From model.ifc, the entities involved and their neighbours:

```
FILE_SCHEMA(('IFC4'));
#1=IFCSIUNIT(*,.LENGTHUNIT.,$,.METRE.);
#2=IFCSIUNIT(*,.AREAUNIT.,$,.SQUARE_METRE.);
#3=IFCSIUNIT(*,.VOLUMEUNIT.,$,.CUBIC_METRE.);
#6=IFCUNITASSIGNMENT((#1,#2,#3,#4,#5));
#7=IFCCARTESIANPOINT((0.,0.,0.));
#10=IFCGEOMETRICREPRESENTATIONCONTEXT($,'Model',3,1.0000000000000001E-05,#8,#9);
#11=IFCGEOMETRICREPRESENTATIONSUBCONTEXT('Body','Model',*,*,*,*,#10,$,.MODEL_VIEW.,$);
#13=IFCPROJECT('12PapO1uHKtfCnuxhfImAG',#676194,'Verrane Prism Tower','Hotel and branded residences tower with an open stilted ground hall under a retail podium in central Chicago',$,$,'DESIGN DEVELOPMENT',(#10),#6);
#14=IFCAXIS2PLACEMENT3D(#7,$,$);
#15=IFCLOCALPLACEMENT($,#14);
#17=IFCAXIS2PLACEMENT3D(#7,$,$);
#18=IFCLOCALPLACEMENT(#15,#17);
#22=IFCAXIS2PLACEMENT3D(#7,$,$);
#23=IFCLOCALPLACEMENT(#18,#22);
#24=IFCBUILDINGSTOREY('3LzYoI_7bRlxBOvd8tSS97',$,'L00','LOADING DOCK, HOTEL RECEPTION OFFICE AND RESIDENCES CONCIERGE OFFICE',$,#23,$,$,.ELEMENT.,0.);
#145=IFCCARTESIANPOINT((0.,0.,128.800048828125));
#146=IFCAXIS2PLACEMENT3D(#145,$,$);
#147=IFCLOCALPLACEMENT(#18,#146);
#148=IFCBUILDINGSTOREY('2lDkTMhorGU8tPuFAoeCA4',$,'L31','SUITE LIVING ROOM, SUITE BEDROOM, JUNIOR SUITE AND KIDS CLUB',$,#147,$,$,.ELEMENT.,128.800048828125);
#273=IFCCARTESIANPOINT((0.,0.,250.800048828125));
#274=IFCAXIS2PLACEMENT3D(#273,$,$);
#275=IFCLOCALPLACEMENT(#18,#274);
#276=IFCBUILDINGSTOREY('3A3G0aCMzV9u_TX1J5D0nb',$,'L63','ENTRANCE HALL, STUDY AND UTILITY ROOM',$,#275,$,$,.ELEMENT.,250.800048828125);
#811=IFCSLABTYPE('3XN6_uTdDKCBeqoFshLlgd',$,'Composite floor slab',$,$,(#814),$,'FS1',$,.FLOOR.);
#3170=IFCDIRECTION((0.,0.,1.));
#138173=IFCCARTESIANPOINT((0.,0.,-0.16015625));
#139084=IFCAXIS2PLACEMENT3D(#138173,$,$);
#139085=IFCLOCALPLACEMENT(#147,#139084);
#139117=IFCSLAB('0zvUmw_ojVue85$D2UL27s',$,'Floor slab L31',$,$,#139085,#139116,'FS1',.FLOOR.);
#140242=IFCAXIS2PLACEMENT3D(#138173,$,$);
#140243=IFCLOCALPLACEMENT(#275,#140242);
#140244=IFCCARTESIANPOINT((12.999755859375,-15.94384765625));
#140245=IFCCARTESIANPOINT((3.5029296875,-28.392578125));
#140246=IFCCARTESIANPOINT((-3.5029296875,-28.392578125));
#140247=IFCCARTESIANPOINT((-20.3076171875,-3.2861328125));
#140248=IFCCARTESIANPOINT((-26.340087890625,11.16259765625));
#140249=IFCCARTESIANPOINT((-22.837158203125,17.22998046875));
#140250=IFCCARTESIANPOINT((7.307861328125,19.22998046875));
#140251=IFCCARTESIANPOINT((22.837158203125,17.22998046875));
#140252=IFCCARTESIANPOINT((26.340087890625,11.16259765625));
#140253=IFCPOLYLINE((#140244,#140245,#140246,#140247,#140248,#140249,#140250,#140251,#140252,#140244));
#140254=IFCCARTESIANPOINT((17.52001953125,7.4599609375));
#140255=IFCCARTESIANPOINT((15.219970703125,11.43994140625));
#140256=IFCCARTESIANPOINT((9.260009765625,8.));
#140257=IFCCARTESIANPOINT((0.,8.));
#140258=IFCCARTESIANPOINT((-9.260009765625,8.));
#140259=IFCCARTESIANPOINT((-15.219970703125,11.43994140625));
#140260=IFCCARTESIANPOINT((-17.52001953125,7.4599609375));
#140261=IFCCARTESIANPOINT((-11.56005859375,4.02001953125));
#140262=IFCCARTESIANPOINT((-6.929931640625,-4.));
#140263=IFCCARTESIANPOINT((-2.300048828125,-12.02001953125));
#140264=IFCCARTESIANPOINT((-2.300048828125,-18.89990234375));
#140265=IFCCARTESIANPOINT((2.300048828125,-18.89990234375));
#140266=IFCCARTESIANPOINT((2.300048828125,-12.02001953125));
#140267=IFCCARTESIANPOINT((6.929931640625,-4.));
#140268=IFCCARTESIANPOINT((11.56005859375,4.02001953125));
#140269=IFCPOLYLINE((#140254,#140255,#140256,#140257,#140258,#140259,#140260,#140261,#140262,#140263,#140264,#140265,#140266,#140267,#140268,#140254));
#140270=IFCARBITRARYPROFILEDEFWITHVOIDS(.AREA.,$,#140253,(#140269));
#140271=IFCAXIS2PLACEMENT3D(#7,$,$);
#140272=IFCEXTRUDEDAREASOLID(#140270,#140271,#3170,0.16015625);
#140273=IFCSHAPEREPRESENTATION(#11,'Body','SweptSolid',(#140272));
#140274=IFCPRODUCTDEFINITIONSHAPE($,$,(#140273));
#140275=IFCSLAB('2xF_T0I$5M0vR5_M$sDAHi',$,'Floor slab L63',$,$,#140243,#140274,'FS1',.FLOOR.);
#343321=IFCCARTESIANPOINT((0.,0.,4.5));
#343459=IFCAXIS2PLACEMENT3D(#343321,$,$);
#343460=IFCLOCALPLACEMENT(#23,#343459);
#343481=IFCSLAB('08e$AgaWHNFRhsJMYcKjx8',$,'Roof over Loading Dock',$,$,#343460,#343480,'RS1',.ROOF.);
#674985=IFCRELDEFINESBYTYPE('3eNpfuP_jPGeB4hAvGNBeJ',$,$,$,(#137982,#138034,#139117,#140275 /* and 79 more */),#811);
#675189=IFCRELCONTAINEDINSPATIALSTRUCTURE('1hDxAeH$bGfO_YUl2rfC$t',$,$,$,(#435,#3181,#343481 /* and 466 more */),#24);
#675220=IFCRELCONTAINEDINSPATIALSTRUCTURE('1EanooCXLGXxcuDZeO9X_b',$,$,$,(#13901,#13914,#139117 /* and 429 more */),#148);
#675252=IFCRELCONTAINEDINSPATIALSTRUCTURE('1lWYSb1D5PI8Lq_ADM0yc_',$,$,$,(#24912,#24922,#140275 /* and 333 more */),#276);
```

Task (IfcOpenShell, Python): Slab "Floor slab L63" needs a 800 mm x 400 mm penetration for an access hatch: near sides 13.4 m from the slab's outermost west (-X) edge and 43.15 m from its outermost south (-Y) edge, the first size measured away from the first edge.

```python
import numpy as np
import ifcopenshell
import ifcopenshell.api.feature
import ifcopenshell.api.geometry
import ifcopenshell.api.root
import ifcopenshell.geom
import ifcopenshell.util.placement
import ifcopenshell.util.representation
import ifcopenshell.util.shape
import ifcopenshell.util.unit

model = ifcopenshell.open("model.ifc")
unit_scale = ifcopenshell.util.unit.calculate_unit_scale(model)
settings = ifcopenshell.geom.settings()


def volume(element):
    """Net volume in cubic metres, openings subtracted."""
    shape = ifcopenshell.geom.create_shape(settings, element)
    return ifcopenshell.util.shape.get_volume(shape.geometry)


slab = model.by_id(140275)
before = volume(slab)

# Extent in the slab's own axes, in metres. The edges named are its -X and -Y sides.
slab_shape = ifcopenshell.geom.create_shape(settings, slab)
vertices = ifcopenshell.util.shape.get_vertices(slab_shape.geometry)
x_min, y_min, bottom = vertices.min(axis=0)
top = vertices[:, 2].max()

opening = ifcopenshell.api.root.create_entity(model, ifc_class="IfcOpeningElement", name="Access hatch opening", predefined_type="OPENING")
context = ifcopenshell.util.representation.get_context(model, "Model", "Body", "MODEL_VIEW")
width, depth = 0.8, 0.4
outline = [(0.0, 0.0), (width, 0.0), (width, depth), (0.0, depth), (0.0, 0.0)]
# Overshoot both faces by 50 mm so the cut is clean.
shape = ifcopenshell.api.geometry.add_slab_representation(
    model, context=context, depth=top - bottom + 0.1, polyline=outline
)
ifcopenshell.api.geometry.assign_representation(model, product=opening, representation=shape)

matrix = ifcopenshell.util.placement.get_local_placement(slab.ObjectPlacement)
matrix[:, 3] = matrix @ np.append(np.array([x_min + 13.4, y_min + 43.15, bottom - 0.05]) / unit_scale, 1.0)
ifcopenshell.api.geometry.edit_object_placement(model, product=opening, matrix=matrix, is_si=False)
ifcopenshell.api.feature.add_feature(model, feature=opening, element=slab)

after = volume(slab)

print(f"slab volume {before:.3f} -> {after:.3f} m3")

model.write("model_edited.ifc")
```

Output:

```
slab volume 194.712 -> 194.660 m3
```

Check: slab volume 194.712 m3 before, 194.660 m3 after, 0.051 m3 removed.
